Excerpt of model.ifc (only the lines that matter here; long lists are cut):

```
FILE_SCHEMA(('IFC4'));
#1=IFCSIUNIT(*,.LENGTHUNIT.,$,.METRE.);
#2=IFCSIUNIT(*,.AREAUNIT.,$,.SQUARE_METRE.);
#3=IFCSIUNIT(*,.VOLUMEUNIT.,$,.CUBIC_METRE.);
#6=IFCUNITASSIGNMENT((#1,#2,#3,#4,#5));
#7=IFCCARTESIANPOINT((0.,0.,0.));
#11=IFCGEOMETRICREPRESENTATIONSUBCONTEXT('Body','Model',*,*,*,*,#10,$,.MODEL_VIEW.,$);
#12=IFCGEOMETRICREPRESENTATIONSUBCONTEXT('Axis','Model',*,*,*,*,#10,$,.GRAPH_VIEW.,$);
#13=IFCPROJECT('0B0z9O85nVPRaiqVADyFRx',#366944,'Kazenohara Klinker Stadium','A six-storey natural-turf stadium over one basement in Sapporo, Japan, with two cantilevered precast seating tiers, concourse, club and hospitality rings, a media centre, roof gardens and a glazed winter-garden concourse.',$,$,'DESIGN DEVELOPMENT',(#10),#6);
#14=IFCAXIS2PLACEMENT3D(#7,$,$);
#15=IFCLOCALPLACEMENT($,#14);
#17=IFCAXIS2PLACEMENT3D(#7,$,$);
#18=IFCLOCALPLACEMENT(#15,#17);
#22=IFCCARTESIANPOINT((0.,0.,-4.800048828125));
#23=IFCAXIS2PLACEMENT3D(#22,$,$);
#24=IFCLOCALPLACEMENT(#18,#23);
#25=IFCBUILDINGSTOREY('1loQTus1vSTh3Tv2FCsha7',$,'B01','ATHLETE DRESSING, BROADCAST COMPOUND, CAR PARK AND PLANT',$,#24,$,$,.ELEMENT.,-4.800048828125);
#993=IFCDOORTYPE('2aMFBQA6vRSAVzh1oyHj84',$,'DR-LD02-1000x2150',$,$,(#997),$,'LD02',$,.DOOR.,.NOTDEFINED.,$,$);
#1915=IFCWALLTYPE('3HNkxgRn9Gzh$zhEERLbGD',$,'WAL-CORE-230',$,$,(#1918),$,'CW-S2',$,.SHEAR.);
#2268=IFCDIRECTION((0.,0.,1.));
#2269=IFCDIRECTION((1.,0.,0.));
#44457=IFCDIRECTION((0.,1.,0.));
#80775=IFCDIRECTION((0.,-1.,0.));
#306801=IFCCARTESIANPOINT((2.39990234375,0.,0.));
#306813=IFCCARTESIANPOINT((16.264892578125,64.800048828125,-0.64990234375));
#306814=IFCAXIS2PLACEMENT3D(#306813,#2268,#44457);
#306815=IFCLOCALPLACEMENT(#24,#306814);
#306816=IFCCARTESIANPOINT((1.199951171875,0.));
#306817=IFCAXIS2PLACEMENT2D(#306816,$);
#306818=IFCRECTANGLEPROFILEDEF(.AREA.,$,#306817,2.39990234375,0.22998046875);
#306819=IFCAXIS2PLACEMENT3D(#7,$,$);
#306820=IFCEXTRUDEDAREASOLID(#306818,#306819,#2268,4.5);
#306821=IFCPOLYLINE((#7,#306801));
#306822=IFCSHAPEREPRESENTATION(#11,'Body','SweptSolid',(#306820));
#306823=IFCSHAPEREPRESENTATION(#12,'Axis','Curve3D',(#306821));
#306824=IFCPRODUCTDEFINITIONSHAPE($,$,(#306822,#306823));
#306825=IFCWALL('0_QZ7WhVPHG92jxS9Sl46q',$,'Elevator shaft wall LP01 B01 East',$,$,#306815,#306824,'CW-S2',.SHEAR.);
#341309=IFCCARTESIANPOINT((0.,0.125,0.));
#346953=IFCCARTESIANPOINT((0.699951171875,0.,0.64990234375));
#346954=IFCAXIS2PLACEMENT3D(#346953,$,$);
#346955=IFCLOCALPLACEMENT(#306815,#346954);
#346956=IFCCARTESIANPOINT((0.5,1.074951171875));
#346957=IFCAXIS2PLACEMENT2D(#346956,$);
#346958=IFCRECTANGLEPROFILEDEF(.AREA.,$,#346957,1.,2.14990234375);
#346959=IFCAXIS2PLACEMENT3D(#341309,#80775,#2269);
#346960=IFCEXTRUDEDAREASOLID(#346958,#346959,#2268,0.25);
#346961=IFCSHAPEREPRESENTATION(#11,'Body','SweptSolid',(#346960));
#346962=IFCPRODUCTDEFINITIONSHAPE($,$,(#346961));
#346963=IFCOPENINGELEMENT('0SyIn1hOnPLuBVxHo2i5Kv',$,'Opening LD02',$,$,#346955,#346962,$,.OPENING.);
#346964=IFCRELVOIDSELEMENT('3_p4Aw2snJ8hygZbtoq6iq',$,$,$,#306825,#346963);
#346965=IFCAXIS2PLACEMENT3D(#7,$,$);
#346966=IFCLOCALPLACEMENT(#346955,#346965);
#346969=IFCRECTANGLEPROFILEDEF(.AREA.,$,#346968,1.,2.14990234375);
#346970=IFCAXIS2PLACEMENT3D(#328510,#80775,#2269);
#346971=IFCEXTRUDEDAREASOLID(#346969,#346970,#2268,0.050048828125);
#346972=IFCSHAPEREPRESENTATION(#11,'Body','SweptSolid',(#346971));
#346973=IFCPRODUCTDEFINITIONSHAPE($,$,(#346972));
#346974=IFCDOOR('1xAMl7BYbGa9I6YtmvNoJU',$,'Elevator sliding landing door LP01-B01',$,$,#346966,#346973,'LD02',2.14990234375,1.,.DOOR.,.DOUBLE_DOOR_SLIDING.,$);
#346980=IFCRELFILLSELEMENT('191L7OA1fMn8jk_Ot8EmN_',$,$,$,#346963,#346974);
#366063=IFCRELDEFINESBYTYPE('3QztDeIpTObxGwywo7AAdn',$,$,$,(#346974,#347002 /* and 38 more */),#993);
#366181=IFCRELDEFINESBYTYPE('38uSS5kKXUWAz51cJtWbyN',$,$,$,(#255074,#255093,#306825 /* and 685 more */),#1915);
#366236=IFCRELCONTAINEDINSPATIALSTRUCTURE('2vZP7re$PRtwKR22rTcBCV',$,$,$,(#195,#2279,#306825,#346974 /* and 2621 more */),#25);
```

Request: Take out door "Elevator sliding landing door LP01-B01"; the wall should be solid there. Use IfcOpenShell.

```python
import ifcopenshell
import ifcopenshell.api.feature
import ifcopenshell.api.root
import ifcopenshell.geom
import ifcopenshell.util.shape

model = ifcopenshell.open("model.ifc")
settings = ifcopenshell.geom.settings()


def volume(element):
    """Net volume in cubic metres, openings subtracted."""
    shape = ifcopenshell.geom.create_shape(settings, element)
    return ifcopenshell.util.shape.get_volume(shape.geometry)


door = model.by_id(346974)
opening = door.FillsVoids[0].RelatingOpeningElement
wall = opening.VoidsElements[0].RelatingBuildingElement
before = volume(wall)

ifcopenshell.api.root.remove_product(model, product=door)
ifcopenshell.api.feature.remove_feature(model, feature=opening)

after = volume(wall)

print(f"wall volume {before:.3f} -> {after:.3f} m3")

model.write("model_updated.ifc")
```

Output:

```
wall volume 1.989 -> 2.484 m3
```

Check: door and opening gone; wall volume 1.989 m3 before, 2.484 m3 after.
